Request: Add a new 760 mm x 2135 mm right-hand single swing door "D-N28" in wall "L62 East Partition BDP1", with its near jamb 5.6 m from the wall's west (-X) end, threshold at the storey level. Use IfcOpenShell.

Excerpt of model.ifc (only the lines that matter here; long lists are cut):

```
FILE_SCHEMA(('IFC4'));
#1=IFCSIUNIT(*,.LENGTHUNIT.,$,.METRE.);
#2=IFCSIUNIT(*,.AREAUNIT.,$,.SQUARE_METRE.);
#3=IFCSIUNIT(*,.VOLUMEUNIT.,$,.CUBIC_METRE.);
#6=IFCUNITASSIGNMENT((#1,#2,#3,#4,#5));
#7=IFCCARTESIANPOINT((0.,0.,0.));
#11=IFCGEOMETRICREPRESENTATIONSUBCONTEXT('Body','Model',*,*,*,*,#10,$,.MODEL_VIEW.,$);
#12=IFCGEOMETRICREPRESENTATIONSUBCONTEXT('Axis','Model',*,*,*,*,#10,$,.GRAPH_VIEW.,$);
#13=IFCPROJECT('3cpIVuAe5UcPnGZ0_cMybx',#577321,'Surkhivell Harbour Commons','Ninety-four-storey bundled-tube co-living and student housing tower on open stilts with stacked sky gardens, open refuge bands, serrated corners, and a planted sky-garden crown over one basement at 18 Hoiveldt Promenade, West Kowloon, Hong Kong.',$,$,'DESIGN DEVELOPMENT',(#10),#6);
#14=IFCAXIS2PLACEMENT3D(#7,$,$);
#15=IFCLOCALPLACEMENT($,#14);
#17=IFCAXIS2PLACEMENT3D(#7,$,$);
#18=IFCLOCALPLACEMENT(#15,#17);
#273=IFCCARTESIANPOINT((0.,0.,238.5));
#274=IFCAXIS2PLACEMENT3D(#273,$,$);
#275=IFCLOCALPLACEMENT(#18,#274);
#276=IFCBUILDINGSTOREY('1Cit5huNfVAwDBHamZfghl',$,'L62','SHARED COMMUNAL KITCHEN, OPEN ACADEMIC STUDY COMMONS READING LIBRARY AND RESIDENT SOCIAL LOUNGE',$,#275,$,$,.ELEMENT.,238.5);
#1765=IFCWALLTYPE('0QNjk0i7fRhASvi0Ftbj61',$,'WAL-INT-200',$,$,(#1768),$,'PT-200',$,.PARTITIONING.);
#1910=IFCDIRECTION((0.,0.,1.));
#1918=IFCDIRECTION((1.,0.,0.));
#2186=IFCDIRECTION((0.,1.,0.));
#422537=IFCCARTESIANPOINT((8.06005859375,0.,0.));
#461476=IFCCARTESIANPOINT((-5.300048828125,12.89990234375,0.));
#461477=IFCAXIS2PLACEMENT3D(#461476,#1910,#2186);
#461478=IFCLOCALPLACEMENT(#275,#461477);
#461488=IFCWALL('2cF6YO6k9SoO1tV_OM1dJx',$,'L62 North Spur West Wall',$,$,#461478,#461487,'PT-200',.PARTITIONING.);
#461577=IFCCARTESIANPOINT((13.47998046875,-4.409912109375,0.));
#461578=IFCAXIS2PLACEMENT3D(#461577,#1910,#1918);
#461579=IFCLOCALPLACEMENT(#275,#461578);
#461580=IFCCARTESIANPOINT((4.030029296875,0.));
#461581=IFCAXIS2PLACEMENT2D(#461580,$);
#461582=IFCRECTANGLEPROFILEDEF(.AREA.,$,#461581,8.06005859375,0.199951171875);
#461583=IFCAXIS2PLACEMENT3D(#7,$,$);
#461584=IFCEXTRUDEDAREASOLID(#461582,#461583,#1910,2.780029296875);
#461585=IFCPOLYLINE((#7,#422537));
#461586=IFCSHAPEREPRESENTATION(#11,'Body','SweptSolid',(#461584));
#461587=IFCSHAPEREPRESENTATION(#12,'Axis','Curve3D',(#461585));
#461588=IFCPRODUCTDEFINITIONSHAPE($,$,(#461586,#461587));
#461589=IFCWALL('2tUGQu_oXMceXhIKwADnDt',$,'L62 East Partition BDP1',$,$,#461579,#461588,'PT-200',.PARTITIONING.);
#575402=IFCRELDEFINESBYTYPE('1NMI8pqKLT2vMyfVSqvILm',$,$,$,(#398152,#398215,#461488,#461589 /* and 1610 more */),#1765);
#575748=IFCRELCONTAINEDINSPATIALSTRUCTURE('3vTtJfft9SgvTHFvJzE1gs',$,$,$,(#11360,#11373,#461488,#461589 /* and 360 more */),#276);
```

```python
import numpy as np
import ifcopenshell
import ifcopenshell.api.feature
import ifcopenshell.api.geometry
import ifcopenshell.api.root
import ifcopenshell.api.spatial
import ifcopenshell.geom
import ifcopenshell.util.element
import ifcopenshell.util.placement
import ifcopenshell.util.representation
import ifcopenshell.util.shape
import ifcopenshell.util.unit

model = ifcopenshell.open("model.ifc")
unit_scale = ifcopenshell.util.unit.calculate_unit_scale(model)
settings = ifcopenshell.geom.settings()


def volume(element):
    """Net volume in cubic metres, openings subtracted."""
    shape = ifcopenshell.geom.create_shape(settings, element)
    return ifcopenshell.util.shape.get_volume(shape.geometry)


wall = model.by_guid("2tUGQu_oXMceXhIKwADnDt")
storey = ifcopenshell.util.element.get_container(wall, ifc_class="IfcBuildingStorey")
context = ifcopenshell.util.representation.get_context(model, "Model", "Body", "MODEL_VIEW")
before = volume(wall)

width, height, from_end, sill = 0.76, 2.135, 5.6, 0.0  # metres

# The wall runs along its own X axis, and the end named is its -X end.
wall_shape = ifcopenshell.geom.create_shape(settings, wall)
x, y, z = ifcopenshell.util.shape.get_vertices(wall_shape.geometry).T
start = x.min() + from_end
face, thickness = float(y.min()), float(y.max() - y.min())
wall_matrix = ifcopenshell.util.placement.get_local_placement(wall.ObjectPlacement)
level = ifcopenshell.util.placement.get_local_placement(storey.ObjectPlacement)[2, 3]


def in_wall(x, y):
    """Placement at x, y metres in the wall's axes, at sill height."""
    matrix = wall_matrix.copy()
    matrix[:, 3] = wall_matrix @ np.array([x / unit_scale, y / unit_scale, 0.0, 1.0])
    matrix[2, 3] = level + sill / unit_scale
    return matrix


# Opening: a box that overshoots both wall faces by 50 mm.
opening = ifcopenshell.api.root.create_entity(model, ifc_class="IfcOpeningElement", predefined_type="OPENING")
box = ifcopenshell.api.geometry.add_wall_representation(
    model, context=context, length=width, height=height, thickness=thickness + 0.1
)
ifcopenshell.api.geometry.assign_representation(model, product=opening, representation=box)
ifcopenshell.api.geometry.edit_object_placement(model, product=opening, matrix=in_wall(start, face - 0.05), is_si=False)
ifcopenshell.api.feature.add_feature(model, feature=opening, element=wall)

door = ifcopenshell.api.root.create_entity(model, ifc_class="IfcDoor", name="D-N28", predefined_type="DOOR")
door.OverallWidth, door.OverallHeight = width / unit_scale, height / unit_scale
door.OperationType = "SINGLE_SWING_RIGHT"
body = ifcopenshell.api.geometry.add_door_representation(
    model,
    context=context,
    overall_width=door.OverallWidth,
    overall_height=door.OverallHeight,
    operation_type="SINGLE_SWING_RIGHT",
    lining_properties={"LiningDepth": thickness / unit_scale, "ThresholdDepth": thickness / unit_scale},
)
ifcopenshell.api.geometry.assign_representation(model, product=door, representation=body)
ifcopenshell.api.spatial.assign_container(model, products=[door], relating_structure=storey)
ifcopenshell.api.feature.add_filling(model, opening=opening, element=door)

# The lining spans the wall, so the door starts at the wall face.
ifcopenshell.api.geometry.edit_object_placement(model, product=door, matrix=in_wall(start, face), is_si=False)

after = volume(wall)

print(f"wall volume {before:.3f} -> {after:.3f} m3")

model.write("model_edited.ifc")
```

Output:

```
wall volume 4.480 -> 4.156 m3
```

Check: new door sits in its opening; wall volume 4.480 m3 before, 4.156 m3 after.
